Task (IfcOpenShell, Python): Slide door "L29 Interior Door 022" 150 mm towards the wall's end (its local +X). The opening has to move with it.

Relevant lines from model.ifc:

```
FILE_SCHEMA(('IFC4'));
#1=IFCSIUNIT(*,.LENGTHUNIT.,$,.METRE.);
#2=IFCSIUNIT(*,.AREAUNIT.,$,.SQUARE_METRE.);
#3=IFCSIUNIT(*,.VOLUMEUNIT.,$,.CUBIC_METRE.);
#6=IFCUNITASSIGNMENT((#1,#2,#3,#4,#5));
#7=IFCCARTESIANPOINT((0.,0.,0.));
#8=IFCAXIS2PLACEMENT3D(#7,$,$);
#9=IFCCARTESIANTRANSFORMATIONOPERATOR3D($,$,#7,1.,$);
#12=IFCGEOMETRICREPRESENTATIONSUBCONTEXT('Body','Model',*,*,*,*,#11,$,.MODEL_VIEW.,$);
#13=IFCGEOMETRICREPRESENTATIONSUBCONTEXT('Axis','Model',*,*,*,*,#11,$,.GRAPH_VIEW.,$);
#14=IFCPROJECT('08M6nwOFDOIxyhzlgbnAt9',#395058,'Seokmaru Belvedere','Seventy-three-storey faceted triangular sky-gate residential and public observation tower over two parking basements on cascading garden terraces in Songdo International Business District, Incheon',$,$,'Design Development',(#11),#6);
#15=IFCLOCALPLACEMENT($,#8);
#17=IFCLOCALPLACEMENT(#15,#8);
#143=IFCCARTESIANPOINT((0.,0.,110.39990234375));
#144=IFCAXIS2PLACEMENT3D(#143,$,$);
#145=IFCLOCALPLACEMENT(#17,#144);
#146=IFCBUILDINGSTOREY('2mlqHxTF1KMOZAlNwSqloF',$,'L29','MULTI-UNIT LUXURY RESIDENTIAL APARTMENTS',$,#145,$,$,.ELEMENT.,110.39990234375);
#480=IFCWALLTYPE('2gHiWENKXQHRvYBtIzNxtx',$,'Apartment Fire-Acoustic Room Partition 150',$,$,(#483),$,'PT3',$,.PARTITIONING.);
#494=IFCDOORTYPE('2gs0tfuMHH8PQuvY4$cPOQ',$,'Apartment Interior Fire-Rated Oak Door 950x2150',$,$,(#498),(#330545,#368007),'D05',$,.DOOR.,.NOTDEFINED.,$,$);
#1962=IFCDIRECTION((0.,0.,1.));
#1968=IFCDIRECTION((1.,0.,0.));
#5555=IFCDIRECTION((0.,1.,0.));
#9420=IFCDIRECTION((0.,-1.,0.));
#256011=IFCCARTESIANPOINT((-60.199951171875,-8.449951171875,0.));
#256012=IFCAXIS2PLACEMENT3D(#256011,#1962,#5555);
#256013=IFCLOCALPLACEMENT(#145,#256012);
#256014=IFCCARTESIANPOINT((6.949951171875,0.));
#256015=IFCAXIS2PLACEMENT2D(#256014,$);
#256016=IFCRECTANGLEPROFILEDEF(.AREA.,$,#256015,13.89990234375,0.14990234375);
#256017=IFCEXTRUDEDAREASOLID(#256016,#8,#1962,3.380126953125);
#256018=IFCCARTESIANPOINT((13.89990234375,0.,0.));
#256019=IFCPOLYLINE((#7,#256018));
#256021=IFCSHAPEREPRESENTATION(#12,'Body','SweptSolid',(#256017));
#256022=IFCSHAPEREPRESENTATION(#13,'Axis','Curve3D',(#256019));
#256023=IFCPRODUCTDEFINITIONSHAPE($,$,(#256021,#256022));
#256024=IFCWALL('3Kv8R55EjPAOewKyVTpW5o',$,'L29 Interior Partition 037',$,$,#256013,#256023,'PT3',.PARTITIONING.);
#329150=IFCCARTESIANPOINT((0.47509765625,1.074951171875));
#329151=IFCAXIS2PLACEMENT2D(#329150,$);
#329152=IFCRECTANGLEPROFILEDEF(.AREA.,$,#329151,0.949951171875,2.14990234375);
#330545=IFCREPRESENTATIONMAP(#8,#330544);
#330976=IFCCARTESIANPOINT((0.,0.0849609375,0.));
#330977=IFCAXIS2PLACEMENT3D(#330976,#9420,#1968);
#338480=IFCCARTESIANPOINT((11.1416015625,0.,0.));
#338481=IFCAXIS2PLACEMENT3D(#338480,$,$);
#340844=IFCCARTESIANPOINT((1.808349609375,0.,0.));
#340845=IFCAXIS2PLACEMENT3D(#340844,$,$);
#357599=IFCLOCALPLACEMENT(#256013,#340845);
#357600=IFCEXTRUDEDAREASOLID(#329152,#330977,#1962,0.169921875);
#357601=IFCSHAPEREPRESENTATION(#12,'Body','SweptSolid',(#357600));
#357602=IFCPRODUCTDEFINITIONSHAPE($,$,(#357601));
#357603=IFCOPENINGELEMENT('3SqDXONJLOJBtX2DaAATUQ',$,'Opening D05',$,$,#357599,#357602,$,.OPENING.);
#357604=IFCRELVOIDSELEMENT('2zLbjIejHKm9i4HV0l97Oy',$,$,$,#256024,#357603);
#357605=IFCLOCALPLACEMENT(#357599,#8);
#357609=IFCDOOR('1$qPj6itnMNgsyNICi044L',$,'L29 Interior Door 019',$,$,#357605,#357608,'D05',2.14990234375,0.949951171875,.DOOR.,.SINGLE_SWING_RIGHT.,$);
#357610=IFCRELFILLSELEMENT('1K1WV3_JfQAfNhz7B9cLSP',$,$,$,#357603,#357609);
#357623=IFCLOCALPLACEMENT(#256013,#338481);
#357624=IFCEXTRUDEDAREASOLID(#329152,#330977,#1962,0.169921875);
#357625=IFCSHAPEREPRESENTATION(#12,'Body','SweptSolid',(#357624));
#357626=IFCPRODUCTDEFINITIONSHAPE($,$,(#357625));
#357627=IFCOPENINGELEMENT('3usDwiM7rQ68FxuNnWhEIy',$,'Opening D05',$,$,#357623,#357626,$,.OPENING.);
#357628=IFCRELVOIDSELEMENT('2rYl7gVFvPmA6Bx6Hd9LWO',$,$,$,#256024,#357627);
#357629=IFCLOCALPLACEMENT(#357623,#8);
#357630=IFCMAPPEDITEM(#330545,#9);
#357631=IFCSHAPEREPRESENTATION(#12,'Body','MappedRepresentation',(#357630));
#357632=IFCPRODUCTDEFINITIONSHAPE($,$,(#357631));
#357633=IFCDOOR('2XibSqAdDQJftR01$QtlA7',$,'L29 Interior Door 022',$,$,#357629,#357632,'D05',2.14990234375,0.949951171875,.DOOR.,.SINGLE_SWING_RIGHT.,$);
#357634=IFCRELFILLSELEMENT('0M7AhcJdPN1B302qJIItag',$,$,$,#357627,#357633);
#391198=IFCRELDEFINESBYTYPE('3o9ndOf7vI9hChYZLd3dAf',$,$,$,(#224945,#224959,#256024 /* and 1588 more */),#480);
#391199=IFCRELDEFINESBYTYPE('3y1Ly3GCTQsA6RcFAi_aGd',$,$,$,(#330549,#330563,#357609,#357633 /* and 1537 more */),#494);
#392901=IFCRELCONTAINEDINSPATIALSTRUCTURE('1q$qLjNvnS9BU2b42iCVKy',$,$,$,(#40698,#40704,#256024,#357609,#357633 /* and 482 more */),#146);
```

```python
import ifcopenshell
import ifcopenshell.api.geometry
import ifcopenshell.util.placement

model = ifcopenshell.open("model.ifc")

door = model.by_guid("2XibSqAdDQJftR01$QtlA7")
opening = door.FillsVoids[0].RelatingOpeningElement
wall = opening.VoidsElements[0].RelatingBuildingElement

wall_matrix = ifcopenshell.util.placement.get_local_placement(wall.ObjectPlacement)
shift = wall_matrix[:3, 0] * 0.15
before = ifcopenshell.util.placement.get_local_placement(door.ObjectPlacement)[:3, 3].copy()

# The door is placed relative to its opening, so it follows when the opening moves.
matrix = ifcopenshell.util.placement.get_local_placement(opening.ObjectPlacement)
matrix[:3, 3] += shift
ifcopenshell.api.geometry.edit_object_placement(
    model, product=opening, matrix=matrix, is_si=False, should_transform_children=True
)

after = ifcopenshell.util.placement.get_local_placement(door.ObjectPlacement)[:3, 3]
print("door moved by", (after - before).round(3) + 0.0)

model.write("model_edited.ifc")
```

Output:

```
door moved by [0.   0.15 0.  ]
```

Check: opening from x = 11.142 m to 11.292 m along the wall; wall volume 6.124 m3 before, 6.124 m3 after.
